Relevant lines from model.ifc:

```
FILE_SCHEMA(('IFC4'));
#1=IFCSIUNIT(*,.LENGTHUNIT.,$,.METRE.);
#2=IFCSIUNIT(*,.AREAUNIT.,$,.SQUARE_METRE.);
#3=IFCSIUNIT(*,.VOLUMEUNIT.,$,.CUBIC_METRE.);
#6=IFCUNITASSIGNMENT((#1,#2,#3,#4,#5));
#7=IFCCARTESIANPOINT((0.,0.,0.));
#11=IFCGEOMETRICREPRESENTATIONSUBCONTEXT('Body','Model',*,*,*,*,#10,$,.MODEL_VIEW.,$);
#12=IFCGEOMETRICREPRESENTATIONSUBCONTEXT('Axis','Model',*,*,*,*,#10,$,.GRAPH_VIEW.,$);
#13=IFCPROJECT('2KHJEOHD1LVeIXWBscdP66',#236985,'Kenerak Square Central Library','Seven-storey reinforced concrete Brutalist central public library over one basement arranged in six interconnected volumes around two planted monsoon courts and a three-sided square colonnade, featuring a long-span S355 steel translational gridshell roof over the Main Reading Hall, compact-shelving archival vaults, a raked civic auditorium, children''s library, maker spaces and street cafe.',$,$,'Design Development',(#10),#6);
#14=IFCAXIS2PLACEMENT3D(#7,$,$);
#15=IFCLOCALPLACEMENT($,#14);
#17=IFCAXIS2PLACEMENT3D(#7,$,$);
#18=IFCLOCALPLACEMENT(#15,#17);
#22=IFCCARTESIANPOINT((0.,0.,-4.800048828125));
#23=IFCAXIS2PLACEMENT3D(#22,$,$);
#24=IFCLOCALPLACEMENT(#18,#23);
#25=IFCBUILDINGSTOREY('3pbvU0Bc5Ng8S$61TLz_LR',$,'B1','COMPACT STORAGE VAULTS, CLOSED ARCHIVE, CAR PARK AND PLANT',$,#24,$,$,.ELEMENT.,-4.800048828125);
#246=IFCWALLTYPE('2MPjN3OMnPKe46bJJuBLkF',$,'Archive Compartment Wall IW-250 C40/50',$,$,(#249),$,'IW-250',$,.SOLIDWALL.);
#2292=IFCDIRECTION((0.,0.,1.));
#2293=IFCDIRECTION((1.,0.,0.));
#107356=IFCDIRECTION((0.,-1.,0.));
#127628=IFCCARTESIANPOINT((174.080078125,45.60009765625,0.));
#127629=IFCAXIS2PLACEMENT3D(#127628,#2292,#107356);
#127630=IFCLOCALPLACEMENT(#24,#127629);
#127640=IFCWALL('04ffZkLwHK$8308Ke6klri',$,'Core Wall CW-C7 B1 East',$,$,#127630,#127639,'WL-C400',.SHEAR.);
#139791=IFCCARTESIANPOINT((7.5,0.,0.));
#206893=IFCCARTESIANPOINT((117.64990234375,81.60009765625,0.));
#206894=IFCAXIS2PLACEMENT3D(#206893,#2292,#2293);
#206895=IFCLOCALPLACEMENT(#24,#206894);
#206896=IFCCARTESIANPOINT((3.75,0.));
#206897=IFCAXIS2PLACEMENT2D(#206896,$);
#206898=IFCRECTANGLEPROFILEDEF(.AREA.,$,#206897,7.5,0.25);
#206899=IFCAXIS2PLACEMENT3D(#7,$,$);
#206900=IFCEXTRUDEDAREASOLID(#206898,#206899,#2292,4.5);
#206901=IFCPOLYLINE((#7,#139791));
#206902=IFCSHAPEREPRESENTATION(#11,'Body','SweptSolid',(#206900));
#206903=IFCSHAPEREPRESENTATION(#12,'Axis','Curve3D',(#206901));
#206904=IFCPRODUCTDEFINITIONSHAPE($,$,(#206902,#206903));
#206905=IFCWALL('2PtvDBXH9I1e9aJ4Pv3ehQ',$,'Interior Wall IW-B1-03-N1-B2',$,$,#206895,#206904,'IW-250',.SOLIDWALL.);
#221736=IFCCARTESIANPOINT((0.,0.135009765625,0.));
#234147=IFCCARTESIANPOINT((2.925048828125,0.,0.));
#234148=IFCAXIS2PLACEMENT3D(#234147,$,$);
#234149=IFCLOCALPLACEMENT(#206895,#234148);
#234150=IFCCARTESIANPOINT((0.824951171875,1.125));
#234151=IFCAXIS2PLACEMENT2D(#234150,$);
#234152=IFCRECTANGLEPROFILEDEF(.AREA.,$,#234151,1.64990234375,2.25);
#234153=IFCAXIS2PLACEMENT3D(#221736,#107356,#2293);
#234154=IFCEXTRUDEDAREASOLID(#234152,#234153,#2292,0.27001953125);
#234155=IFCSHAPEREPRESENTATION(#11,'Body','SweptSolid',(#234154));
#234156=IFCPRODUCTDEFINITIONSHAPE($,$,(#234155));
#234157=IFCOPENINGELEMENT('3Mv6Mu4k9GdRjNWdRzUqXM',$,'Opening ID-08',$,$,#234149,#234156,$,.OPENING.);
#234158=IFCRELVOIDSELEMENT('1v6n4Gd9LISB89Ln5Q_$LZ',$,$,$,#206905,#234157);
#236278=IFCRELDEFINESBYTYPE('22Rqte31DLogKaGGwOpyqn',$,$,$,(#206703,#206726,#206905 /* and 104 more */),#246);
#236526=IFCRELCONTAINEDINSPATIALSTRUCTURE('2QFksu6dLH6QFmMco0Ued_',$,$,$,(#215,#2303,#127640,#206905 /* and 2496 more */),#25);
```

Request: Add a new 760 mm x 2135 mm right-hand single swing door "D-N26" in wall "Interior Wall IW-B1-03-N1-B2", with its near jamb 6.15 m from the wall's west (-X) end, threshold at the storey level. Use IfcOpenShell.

```python
import numpy as np
import ifcopenshell
import ifcopenshell.api.feature
import ifcopenshell.api.geometry
import ifcopenshell.api.root
import ifcopenshell.api.spatial
import ifcopenshell.geom
import ifcopenshell.util.element
import ifcopenshell.util.placement
import ifcopenshell.util.representation
import ifcopenshell.util.shape
import ifcopenshell.util.unit

model = ifcopenshell.open("model.ifc")
unit_scale = ifcopenshell.util.unit.calculate_unit_scale(model)
settings = ifcopenshell.geom.settings()


def volume(element):
    """Net volume in cubic metres, openings subtracted."""
    shape = ifcopenshell.geom.create_shape(settings, element)
    return ifcopenshell.util.shape.get_volume(shape.geometry)


wall = model.by_guid("2PtvDBXH9I1e9aJ4Pv3ehQ")
storey = ifcopenshell.util.element.get_container(wall, ifc_class="IfcBuildingStorey")
context = ifcopenshell.util.representation.get_context(model, "Model", "Body", "MODEL_VIEW")
before = volume(wall)

width, height, from_end, sill = 0.76, 2.135, 6.15, 0.0  # metres

# The wall runs along its own X axis, and the end named is its -X end.
wall_shape = ifcopenshell.geom.create_shape(settings, wall)
x, y, z = ifcopenshell.util.shape.get_vertices(wall_shape.geometry).T
start = x.min() + from_end
face, thickness = float(y.min()), float(y.max() - y.min())
wall_matrix = ifcopenshell.util.placement.get_local_placement(wall.ObjectPlacement)
level = ifcopenshell.util.placement.get_local_placement(storey.ObjectPlacement)[2, 3]


def in_wall(x, y):
    """Placement at x, y metres in the wall's axes, at sill height."""
    matrix = wall_matrix.copy()
    matrix[:, 3] = wall_matrix @ np.array([x / unit_scale, y / unit_scale, 0.0, 1.0])
    matrix[2, 3] = level + sill / unit_scale
    return matrix


# Opening: a box that overshoots both wall faces by 50 mm.
opening = ifcopenshell.api.root.create_entity(model, ifc_class="IfcOpeningElement", predefined_type="OPENING")
box = ifcopenshell.api.geometry.add_wall_representation(
    model, context=context, length=width, height=height, thickness=thickness + 0.1
)
ifcopenshell.api.geometry.assign_representation(model, product=opening, representation=box)
ifcopenshell.api.geometry.edit_object_placement(model, product=opening, matrix=in_wall(start, face - 0.05), is_si=False)
ifcopenshell.api.feature.add_feature(model, feature=opening, element=wall)

door = ifcopenshell.api.root.create_entity(model, ifc_class="IfcDoor", name="D-N26", predefined_type="DOOR")
door.OverallWidth, door.OverallHeight = width / unit_scale, height / unit_scale
door.OperationType = "SINGLE_SWING_RIGHT"
body = ifcopenshell.api.geometry.add_door_representation(
    model,
    context=context,
    overall_width=door.OverallWidth,
    overall_height=door.OverallHeight,
    operation_type="SINGLE_SWING_RIGHT",
    lining_properties={"LiningDepth": thickness / unit_scale, "ThresholdDepth": thickness / unit_scale},
)
ifcopenshell.api.geometry.assign_representation(model, product=door, representation=body)
ifcopenshell.api.spatial.assign_container(model, products=[door], relating_structure=storey)
ifcopenshell.api.feature.add_filling(model, opening=opening, element=door)

# The lining spans the wall, so the door starts at the wall face.
ifcopenshell.api.geometry.edit_object_placement(model, product=door, matrix=in_wall(start, face), is_si=False)

after = volume(wall)

print(f"wall volume {before:.3f} -> {after:.3f} m3")

model.write("model-out.ifc")
```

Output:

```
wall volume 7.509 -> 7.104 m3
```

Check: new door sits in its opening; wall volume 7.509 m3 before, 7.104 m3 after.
